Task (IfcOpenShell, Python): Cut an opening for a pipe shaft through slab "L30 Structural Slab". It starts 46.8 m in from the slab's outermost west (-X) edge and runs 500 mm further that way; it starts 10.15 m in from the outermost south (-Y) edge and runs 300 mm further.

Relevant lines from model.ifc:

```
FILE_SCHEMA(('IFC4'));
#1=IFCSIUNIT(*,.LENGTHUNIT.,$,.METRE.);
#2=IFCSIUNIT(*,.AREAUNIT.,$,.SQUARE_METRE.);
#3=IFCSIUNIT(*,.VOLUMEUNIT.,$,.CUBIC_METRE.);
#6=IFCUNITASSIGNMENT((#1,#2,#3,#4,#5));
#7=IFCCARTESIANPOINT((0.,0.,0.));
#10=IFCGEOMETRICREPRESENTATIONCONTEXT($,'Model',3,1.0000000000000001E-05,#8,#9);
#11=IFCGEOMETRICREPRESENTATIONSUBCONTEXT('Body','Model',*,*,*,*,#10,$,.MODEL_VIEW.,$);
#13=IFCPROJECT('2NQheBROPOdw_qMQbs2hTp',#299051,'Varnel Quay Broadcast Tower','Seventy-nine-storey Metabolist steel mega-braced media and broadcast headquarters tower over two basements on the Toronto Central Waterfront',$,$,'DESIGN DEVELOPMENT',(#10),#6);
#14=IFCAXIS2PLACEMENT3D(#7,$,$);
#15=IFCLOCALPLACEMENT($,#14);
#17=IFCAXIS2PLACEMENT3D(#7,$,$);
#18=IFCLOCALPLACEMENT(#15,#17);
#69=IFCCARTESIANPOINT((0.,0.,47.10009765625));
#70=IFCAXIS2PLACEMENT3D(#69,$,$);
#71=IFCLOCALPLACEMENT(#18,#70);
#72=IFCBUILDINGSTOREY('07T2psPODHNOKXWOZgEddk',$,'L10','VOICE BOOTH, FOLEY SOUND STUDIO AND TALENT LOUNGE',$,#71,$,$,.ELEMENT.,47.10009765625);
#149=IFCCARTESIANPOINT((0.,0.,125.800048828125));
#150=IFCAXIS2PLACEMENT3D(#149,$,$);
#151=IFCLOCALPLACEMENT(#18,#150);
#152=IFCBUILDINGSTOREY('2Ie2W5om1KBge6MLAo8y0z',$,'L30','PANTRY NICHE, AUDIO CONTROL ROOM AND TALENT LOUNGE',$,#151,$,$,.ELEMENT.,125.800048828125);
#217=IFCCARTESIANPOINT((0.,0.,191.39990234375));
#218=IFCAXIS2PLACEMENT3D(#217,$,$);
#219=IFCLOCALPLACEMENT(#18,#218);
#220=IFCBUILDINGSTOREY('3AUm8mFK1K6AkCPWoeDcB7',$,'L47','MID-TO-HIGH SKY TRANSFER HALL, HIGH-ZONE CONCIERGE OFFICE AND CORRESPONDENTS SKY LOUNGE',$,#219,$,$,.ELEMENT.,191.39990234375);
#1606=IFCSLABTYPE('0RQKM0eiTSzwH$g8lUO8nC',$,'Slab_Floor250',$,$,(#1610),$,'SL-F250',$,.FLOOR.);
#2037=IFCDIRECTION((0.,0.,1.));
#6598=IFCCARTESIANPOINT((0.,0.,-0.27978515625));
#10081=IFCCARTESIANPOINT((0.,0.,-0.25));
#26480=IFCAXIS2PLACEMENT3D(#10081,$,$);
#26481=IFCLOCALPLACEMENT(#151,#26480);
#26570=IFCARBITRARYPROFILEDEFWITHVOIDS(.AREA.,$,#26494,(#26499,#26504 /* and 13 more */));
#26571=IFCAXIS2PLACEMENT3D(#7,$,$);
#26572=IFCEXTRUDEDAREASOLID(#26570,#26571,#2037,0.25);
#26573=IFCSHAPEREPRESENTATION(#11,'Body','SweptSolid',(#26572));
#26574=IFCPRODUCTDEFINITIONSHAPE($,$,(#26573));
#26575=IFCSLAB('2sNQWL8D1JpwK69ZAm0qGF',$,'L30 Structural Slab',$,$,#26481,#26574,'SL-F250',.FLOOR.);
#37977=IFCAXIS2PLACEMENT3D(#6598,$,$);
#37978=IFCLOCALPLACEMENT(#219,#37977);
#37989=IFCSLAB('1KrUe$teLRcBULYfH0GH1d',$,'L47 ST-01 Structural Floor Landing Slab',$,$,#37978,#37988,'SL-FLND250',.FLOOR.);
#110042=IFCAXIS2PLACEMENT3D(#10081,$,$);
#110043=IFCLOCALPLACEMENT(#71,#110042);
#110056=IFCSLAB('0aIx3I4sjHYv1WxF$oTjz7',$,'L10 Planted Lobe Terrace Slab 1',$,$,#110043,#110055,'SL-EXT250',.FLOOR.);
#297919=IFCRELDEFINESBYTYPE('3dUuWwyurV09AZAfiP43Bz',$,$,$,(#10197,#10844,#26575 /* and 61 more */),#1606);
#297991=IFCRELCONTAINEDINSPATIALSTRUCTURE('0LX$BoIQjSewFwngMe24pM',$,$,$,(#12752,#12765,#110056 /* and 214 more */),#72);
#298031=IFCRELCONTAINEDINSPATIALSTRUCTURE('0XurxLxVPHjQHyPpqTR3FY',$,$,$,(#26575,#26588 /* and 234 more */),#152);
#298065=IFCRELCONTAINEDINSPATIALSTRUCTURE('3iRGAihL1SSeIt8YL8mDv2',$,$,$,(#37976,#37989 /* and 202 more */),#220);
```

```python
import numpy as np
import ifcopenshell
import ifcopenshell.api.feature
import ifcopenshell.api.geometry
import ifcopenshell.api.root
import ifcopenshell.geom
import ifcopenshell.util.placement
import ifcopenshell.util.representation
import ifcopenshell.util.shape
import ifcopenshell.util.unit

model = ifcopenshell.open("model.ifc")
unit_scale = ifcopenshell.util.unit.calculate_unit_scale(model)
settings = ifcopenshell.geom.settings()


def volume(element):
    """Net volume in cubic metres, openings subtracted."""
    shape = ifcopenshell.geom.create_shape(settings, element)
    return ifcopenshell.util.shape.get_volume(shape.geometry)


slab = model.by_id(26575)
before = volume(slab)

# Extent in the slab's own axes, in metres. The edges named are its -X and -Y sides.
slab_shape = ifcopenshell.geom.create_shape(settings, slab)
vertices = ifcopenshell.util.shape.get_vertices(slab_shape.geometry)
x_min, y_min, bottom = vertices.min(axis=0)
top = vertices[:, 2].max()

opening = ifcopenshell.api.root.create_entity(model, ifc_class="IfcOpeningElement", name="Pipe shaft opening", predefined_type="OPENING")
context = ifcopenshell.util.representation.get_context(model, "Model", "Body", "MODEL_VIEW")
width, depth = 0.5, 0.3
outline = [(0.0, 0.0), (width, 0.0), (width, depth), (0.0, depth), (0.0, 0.0)]
# Overshoot both faces by 50 mm so the cut is clean.
shape = ifcopenshell.api.geometry.add_slab_representation(
    model, context=context, depth=top - bottom + 0.1, polyline=outline
)
ifcopenshell.api.geometry.assign_representation(model, product=opening, representation=shape)

matrix = ifcopenshell.util.placement.get_local_placement(slab.ObjectPlacement)
matrix[:, 3] = matrix @ np.append(np.array([x_min + 46.8, y_min + 10.15, bottom - 0.05]) / unit_scale, 1.0)
ifcopenshell.api.geometry.edit_object_placement(model, product=opening, matrix=matrix, is_si=False)
ifcopenshell.api.feature.add_feature(model, feature=opening, element=slab)

after = volume(slab)

print(f"slab volume {before:.3f} -> {after:.3f} m3")

model.write("model_edited.ifc")
```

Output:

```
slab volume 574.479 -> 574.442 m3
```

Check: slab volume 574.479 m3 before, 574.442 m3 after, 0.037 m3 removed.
